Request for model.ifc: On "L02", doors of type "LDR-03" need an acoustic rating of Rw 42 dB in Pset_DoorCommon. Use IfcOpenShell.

First a look at what the model holds.

```python
import ifcopenshell
import ifcopenshell.util.element

model = ifcopenshell.open("model.ifc")
print(model.schema)
storey = next(s for s in model.by_type("IfcBuildingStorey") if s.Name == "L02")
doors = [e for e in ifcopenshell.util.element.get_decomposition(storey) if e.is_a("IfcDoor")]
seen = {}
for e in doors:
    element_type = ifcopenshell.util.element.get_type(e)
    key = (element_type.Name if element_type != e and element_type else None, ifcopenshell.util.element.get_pset(e, "Pset_DoorCommon", "AcousticRating"))
    seen[key] = seen.get(key, 0) + 1
for (name, value), count in sorted(seen.items(), key=str):
    print(count, "x", name, "|", value)
```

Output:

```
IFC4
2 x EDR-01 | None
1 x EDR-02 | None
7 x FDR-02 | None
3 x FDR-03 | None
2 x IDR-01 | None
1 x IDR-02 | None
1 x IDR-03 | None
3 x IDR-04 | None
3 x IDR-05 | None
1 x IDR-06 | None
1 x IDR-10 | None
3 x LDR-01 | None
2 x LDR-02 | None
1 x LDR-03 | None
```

```python
import ifcopenshell
import ifcopenshell.api.pset
import ifcopenshell.util.element

model = ifcopenshell.open("model.ifc")

storey = next(s for s in model.by_type("IfcBuildingStorey") if s.Name == "L02")
doors = [e for e in ifcopenshell.util.element.get_decomposition(storey) if e.is_a("IfcDoor")]

count = 0
for e in doors:
    element_type = ifcopenshell.util.element.get_type(e)
    if element_type in (None, e) or element_type.Name != "LDR-03":
        continue
    # add_pset returns the element's existing set when there is one.
    pset = ifcopenshell.api.pset.add_pset(model, product=e, name="Pset_DoorCommon")
    ifcopenshell.api.pset.edit_pset(model, pset=pset, properties={"AcousticRating": "Rw 42 dB"})
    count += 1

print(count, "doors updated")

model.write("model_rev.ifc")
```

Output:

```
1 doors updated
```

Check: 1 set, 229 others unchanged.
